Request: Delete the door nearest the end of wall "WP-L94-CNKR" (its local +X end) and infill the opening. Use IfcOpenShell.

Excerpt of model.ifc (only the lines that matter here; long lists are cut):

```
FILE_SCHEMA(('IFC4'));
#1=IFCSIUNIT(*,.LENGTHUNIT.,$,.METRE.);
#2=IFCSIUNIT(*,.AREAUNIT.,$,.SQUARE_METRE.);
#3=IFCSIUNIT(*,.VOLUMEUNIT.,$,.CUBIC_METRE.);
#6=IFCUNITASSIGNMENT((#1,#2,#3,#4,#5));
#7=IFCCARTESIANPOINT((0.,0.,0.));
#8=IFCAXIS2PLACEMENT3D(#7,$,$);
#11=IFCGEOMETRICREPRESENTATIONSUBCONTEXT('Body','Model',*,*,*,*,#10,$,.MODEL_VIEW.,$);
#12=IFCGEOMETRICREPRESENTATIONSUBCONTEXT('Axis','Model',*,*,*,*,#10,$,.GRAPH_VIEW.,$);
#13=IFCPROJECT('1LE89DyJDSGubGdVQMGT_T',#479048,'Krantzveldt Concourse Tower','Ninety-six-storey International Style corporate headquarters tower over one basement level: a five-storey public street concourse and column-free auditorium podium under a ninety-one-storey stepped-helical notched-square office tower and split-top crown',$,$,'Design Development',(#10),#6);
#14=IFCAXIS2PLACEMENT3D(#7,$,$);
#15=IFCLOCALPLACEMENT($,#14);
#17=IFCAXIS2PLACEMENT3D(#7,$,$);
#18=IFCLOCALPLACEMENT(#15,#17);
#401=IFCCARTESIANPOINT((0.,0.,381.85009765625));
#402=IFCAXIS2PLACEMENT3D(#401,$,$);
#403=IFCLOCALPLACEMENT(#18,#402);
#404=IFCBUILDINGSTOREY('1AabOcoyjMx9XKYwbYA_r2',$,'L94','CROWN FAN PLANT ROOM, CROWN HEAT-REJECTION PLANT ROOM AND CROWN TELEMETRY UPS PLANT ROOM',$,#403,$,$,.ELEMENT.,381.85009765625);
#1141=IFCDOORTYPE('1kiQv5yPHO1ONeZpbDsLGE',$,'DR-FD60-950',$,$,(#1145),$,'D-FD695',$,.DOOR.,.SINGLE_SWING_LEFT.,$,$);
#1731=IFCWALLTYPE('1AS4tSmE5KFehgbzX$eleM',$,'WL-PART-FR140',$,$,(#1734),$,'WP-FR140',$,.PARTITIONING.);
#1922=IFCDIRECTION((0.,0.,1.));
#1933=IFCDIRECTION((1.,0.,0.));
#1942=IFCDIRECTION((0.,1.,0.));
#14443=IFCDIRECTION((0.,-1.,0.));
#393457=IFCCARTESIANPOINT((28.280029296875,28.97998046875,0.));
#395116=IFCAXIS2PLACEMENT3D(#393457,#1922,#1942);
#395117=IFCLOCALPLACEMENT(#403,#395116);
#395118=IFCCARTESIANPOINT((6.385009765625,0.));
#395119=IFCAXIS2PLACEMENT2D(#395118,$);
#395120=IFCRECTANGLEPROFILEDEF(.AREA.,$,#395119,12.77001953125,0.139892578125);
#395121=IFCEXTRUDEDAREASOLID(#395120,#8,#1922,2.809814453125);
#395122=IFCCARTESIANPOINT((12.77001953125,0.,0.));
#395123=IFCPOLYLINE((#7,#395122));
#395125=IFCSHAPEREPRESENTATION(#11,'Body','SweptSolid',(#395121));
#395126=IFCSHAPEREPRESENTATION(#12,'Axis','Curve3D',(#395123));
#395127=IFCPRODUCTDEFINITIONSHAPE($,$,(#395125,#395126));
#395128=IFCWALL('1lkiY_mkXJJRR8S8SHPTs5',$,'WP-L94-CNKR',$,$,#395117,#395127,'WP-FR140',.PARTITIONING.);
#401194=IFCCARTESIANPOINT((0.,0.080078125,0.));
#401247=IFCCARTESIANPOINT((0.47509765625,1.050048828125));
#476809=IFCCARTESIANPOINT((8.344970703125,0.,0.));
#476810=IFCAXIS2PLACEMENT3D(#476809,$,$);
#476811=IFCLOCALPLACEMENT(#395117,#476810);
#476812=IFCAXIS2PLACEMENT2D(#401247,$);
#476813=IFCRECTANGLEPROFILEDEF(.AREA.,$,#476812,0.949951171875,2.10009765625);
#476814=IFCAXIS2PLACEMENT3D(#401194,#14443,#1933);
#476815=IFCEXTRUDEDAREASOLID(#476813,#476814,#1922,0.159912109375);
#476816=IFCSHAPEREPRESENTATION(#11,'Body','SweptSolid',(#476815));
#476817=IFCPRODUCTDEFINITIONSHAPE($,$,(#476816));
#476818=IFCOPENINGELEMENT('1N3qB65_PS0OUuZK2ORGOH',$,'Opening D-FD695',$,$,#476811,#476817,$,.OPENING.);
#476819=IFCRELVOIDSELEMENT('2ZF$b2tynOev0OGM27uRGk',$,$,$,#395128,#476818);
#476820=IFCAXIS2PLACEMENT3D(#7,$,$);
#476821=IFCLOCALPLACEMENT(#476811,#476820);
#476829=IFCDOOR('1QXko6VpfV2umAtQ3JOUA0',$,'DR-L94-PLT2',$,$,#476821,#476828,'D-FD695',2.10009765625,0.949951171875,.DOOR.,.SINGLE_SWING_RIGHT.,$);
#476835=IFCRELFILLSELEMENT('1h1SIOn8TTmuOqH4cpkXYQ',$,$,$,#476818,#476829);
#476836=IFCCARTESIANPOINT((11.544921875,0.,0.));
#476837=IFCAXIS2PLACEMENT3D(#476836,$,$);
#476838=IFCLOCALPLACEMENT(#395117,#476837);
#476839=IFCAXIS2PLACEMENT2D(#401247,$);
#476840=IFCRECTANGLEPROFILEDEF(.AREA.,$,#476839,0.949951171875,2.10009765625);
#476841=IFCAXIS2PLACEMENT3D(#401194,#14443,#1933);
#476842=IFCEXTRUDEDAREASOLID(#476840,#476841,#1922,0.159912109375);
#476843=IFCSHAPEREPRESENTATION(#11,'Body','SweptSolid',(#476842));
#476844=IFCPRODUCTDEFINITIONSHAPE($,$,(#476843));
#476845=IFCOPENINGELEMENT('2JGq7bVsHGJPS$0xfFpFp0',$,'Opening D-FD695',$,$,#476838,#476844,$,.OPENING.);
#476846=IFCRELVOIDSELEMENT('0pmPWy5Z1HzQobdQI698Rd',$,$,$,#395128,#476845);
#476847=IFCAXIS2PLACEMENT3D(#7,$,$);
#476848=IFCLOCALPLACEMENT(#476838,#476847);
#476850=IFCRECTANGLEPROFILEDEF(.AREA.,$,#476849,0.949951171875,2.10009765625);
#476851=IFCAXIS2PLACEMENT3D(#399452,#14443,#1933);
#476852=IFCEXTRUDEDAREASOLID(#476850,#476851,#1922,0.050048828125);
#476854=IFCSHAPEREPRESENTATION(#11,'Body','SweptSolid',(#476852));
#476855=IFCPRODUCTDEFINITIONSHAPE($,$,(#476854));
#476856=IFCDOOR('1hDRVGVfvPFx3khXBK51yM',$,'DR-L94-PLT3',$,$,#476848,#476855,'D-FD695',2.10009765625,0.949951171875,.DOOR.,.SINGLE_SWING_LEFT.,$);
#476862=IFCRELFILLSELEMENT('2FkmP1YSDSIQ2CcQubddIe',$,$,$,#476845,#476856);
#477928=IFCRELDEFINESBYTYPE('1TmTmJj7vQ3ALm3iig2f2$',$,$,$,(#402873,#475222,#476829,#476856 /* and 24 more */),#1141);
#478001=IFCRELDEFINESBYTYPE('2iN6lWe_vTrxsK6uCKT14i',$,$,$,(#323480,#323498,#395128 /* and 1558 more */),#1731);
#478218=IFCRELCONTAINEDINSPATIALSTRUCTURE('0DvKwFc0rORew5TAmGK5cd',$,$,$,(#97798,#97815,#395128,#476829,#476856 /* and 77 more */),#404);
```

```python
import ifcopenshell
import ifcopenshell.api.feature
import ifcopenshell.api.root
import ifcopenshell.geom
import ifcopenshell.util.shape

model = ifcopenshell.open("model.ifc")
settings = ifcopenshell.geom.settings()


def volume(element):
    """Net volume in cubic metres, openings subtracted."""
    shape = ifcopenshell.geom.create_shape(settings, element)
    return ifcopenshell.util.shape.get_volume(shape.geometry)


door = model.by_id(476856)
opening = door.FillsVoids[0].RelatingOpeningElement
wall = opening.VoidsElements[0].RelatingBuildingElement
before = volume(wall)

ifcopenshell.api.root.remove_product(model, product=door)
ifcopenshell.api.feature.remove_feature(model, feature=opening)

after = volume(wall)

print(f"wall volume {before:.3f} -> {after:.3f} m3")

model.write("model-out.ifc")
```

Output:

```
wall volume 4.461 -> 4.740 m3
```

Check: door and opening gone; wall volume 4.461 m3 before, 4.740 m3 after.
